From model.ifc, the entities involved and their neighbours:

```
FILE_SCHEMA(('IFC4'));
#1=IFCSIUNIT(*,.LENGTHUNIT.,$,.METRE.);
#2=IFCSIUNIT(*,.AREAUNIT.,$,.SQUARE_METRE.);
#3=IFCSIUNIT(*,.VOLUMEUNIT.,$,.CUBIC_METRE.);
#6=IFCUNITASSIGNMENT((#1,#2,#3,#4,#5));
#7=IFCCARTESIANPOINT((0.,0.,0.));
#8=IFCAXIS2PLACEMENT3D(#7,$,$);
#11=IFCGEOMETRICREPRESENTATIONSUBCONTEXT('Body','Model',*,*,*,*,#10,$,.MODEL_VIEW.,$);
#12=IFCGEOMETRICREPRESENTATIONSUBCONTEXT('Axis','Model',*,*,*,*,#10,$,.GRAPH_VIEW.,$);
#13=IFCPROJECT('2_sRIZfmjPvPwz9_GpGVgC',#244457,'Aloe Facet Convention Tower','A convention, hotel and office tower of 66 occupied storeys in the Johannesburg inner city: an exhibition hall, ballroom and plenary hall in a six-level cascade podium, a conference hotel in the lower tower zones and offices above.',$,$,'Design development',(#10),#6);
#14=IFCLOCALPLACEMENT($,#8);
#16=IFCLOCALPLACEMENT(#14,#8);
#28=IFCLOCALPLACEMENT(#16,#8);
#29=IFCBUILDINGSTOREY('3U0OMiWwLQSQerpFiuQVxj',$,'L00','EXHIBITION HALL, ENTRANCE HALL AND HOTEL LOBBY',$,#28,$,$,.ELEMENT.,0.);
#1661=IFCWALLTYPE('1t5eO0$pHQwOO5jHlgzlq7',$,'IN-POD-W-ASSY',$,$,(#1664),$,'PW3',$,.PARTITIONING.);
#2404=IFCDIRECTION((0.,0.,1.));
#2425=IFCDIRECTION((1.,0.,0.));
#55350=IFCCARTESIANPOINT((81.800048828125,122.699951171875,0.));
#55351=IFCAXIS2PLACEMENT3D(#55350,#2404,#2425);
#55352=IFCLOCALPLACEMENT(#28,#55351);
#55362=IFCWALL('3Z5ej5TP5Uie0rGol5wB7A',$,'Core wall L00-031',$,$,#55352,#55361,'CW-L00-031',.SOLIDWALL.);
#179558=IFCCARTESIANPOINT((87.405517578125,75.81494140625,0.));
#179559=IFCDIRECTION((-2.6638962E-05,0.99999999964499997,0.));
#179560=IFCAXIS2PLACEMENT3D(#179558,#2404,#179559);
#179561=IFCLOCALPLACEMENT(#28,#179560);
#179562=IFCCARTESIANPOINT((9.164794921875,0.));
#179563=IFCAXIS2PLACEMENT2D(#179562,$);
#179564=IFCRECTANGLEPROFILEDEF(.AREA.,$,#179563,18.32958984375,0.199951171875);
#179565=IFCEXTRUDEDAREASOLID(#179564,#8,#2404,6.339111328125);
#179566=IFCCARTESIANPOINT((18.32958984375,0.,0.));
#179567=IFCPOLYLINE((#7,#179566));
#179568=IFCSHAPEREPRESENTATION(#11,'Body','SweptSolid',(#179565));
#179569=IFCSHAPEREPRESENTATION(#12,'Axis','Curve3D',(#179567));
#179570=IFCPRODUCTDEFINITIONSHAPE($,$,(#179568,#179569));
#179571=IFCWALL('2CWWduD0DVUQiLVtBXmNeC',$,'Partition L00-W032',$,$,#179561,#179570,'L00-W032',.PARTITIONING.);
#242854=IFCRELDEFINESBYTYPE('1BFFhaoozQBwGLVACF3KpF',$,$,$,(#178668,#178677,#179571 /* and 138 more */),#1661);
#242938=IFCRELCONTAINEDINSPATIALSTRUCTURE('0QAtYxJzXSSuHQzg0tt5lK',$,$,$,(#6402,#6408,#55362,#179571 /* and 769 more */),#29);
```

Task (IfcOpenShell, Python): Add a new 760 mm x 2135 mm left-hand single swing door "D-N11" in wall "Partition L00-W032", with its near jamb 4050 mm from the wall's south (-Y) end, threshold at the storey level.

```python
import numpy as np
import ifcopenshell
import ifcopenshell.api.feature
import ifcopenshell.api.geometry
import ifcopenshell.api.root
import ifcopenshell.api.spatial
import ifcopenshell.geom
import ifcopenshell.util.element
import ifcopenshell.util.placement
import ifcopenshell.util.representation
import ifcopenshell.util.shape
import ifcopenshell.util.unit

model = ifcopenshell.open("model.ifc")
unit_scale = ifcopenshell.util.unit.calculate_unit_scale(model)
settings = ifcopenshell.geom.settings()


def volume(element):
    """Net volume in cubic metres, openings subtracted."""
    shape = ifcopenshell.geom.create_shape(settings, element)
    return ifcopenshell.util.shape.get_volume(shape.geometry)


wall = model.by_id(179571)
storey = ifcopenshell.util.element.get_container(wall, ifc_class="IfcBuildingStorey")
context = ifcopenshell.util.representation.get_context(model, "Model", "Body", "MODEL_VIEW")
before = volume(wall)

width, height, from_end, sill = 0.76, 2.135, 4.05, 0.0  # metres

# The wall runs along its own X axis, and the end named is its -X end.
wall_shape = ifcopenshell.geom.create_shape(settings, wall)
x, y, z = ifcopenshell.util.shape.get_vertices(wall_shape.geometry).T
start = x.min() + from_end
face, thickness = float(y.min()), float(y.max() - y.min())
wall_matrix = ifcopenshell.util.placement.get_local_placement(wall.ObjectPlacement)
level = ifcopenshell.util.placement.get_local_placement(storey.ObjectPlacement)[2, 3]


def in_wall(x, y):
    """Placement at x, y metres in the wall's axes, at sill height."""
    matrix = wall_matrix.copy()
    matrix[:, 3] = wall_matrix @ np.array([x / unit_scale, y / unit_scale, 0.0, 1.0])
    matrix[2, 3] = level + sill / unit_scale
    return matrix


# Opening: a box that overshoots both wall faces by 50 mm.
opening = ifcopenshell.api.root.create_entity(model, ifc_class="IfcOpeningElement", predefined_type="OPENING")
box = ifcopenshell.api.geometry.add_wall_representation(
    model, context=context, length=width, height=height, thickness=thickness + 0.1
)
ifcopenshell.api.geometry.assign_representation(model, product=opening, representation=box)
ifcopenshell.api.geometry.edit_object_placement(model, product=opening, matrix=in_wall(start, face - 0.05), is_si=False)
ifcopenshell.api.feature.add_feature(model, feature=opening, element=wall)

door = ifcopenshell.api.root.create_entity(model, ifc_class="IfcDoor", name="D-N11", predefined_type="DOOR")
door.OverallWidth, door.OverallHeight = width / unit_scale, height / unit_scale
door.OperationType = "SINGLE_SWING_LEFT"
body = ifcopenshell.api.geometry.add_door_representation(
    model,
    context=context,
    overall_width=door.OverallWidth,
    overall_height=door.OverallHeight,
    operation_type="SINGLE_SWING_LEFT",
    lining_properties={"LiningDepth": thickness / unit_scale, "ThresholdDepth": thickness / unit_scale},
)
ifcopenshell.api.geometry.assign_representation(model, product=door, representation=body)
ifcopenshell.api.spatial.assign_container(model, products=[door], relating_structure=storey)
ifcopenshell.api.feature.add_filling(model, opening=opening, element=door)

# The lining spans the wall, so the door starts at the wall face.
ifcopenshell.api.geometry.edit_object_placement(model, product=door, matrix=in_wall(start, face), is_si=False)

after = volume(wall)

print(f"wall volume {before:.3f} -> {after:.3f} m3")

model.write("model-out.ifc")
```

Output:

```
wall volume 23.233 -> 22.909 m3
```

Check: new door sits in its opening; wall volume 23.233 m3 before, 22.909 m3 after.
